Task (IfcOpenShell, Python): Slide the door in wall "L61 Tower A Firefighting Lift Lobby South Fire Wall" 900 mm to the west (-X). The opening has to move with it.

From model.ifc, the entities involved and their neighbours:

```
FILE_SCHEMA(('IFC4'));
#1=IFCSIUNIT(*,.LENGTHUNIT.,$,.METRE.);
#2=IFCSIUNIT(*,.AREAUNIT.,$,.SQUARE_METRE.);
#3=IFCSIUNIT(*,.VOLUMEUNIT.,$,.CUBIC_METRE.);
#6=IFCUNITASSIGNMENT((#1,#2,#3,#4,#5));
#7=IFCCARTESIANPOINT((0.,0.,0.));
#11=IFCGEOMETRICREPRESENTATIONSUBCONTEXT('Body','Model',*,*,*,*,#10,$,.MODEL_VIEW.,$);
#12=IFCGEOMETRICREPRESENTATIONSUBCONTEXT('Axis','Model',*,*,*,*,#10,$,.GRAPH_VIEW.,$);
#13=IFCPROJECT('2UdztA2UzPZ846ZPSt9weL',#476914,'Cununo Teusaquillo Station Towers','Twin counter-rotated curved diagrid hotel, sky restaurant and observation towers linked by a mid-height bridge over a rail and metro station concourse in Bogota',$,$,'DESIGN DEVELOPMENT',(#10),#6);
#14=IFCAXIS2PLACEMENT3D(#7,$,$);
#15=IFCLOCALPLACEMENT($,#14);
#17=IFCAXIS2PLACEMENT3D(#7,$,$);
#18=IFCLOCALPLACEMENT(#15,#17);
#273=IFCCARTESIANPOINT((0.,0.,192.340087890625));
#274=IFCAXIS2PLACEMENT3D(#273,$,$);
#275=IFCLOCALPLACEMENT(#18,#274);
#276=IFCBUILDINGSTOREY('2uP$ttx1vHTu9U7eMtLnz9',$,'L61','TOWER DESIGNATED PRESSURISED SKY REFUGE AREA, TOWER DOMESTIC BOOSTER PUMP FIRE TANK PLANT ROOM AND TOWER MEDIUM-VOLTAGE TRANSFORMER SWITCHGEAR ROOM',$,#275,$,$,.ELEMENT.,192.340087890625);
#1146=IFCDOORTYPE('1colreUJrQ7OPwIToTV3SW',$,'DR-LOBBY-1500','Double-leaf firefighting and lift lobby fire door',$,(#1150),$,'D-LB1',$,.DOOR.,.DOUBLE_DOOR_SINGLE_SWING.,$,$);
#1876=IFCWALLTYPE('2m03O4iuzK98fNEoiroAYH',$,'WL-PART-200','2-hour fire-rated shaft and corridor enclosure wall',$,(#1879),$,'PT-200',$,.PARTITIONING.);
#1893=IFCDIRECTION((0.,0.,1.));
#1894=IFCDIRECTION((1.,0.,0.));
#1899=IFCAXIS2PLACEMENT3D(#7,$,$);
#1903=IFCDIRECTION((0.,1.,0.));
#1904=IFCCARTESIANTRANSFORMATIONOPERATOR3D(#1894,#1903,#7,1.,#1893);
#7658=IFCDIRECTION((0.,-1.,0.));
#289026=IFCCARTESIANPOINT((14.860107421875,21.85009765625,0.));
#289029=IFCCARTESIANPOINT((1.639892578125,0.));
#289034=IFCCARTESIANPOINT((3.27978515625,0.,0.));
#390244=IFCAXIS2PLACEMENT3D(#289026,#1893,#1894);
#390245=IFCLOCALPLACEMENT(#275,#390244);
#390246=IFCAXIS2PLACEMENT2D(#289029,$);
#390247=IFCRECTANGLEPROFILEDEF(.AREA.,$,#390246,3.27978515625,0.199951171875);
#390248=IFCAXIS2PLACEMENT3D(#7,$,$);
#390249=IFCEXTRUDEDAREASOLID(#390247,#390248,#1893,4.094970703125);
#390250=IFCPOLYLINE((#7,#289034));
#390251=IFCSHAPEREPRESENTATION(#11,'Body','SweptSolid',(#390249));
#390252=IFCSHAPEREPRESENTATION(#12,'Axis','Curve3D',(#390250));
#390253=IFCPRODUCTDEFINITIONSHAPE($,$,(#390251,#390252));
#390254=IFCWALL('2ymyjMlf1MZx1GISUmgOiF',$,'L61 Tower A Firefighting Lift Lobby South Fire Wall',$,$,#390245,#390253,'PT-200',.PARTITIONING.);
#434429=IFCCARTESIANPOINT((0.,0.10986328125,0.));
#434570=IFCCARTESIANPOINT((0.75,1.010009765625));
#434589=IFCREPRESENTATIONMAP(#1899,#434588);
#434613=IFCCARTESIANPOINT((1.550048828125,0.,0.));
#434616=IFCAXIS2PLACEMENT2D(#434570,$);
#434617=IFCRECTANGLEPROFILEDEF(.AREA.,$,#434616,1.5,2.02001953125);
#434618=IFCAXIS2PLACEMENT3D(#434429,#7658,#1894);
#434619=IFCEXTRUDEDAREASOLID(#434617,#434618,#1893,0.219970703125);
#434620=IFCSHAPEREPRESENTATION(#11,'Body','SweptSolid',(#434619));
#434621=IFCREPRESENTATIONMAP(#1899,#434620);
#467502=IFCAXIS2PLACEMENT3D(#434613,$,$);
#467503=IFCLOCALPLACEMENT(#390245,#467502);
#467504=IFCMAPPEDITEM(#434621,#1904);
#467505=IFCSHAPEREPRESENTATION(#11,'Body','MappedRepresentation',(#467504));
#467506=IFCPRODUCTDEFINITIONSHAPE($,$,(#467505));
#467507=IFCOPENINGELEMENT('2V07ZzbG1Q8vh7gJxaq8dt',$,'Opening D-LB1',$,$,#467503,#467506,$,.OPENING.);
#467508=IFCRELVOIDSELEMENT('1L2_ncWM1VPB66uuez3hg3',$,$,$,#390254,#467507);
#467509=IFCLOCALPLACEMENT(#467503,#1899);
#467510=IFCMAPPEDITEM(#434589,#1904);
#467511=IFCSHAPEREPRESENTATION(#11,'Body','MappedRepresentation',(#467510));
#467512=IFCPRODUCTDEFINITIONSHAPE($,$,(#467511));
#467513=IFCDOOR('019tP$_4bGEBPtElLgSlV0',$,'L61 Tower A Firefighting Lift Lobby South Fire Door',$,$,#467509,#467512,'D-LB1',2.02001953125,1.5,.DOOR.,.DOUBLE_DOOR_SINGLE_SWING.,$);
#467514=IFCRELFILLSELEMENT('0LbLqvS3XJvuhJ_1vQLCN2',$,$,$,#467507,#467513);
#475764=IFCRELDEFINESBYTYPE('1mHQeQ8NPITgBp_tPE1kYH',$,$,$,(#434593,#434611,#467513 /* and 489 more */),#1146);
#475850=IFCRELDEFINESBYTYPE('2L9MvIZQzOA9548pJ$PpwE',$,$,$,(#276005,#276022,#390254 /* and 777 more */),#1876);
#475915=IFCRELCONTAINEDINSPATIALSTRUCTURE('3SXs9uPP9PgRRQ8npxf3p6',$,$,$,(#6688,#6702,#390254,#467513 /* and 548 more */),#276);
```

```python
import ifcopenshell
import ifcopenshell.api.geometry
import ifcopenshell.util.placement
import ifcopenshell.util.unit

model = ifcopenshell.open("model.ifc")
unit_scale = ifcopenshell.util.unit.calculate_unit_scale(model)

door = model.by_guid("019tP$_4bGEBPtElLgSlV0")
opening = door.FillsVoids[0].RelatingOpeningElement
wall = opening.VoidsElements[0].RelatingBuildingElement

wall_matrix = ifcopenshell.util.placement.get_local_placement(wall.ObjectPlacement)
shift = wall_matrix[:3, 0] * -0.9 / unit_scale
before = ifcopenshell.util.placement.get_local_placement(door.ObjectPlacement)[:3, 3].copy()

# The door is placed relative to its opening, so it follows when the opening moves.
matrix = ifcopenshell.util.placement.get_local_placement(opening.ObjectPlacement)
matrix[:3, 3] += shift
ifcopenshell.api.geometry.edit_object_placement(
    model, product=opening, matrix=matrix, is_si=False, should_transform_children=True
)

after = ifcopenshell.util.placement.get_local_placement(door.ObjectPlacement)[:3, 3]
print("door moved by", (after - before).round(3) + 0.0)

model.write("model_v2.ifc")
```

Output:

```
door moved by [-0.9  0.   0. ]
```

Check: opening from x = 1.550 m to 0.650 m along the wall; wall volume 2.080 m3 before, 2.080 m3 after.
